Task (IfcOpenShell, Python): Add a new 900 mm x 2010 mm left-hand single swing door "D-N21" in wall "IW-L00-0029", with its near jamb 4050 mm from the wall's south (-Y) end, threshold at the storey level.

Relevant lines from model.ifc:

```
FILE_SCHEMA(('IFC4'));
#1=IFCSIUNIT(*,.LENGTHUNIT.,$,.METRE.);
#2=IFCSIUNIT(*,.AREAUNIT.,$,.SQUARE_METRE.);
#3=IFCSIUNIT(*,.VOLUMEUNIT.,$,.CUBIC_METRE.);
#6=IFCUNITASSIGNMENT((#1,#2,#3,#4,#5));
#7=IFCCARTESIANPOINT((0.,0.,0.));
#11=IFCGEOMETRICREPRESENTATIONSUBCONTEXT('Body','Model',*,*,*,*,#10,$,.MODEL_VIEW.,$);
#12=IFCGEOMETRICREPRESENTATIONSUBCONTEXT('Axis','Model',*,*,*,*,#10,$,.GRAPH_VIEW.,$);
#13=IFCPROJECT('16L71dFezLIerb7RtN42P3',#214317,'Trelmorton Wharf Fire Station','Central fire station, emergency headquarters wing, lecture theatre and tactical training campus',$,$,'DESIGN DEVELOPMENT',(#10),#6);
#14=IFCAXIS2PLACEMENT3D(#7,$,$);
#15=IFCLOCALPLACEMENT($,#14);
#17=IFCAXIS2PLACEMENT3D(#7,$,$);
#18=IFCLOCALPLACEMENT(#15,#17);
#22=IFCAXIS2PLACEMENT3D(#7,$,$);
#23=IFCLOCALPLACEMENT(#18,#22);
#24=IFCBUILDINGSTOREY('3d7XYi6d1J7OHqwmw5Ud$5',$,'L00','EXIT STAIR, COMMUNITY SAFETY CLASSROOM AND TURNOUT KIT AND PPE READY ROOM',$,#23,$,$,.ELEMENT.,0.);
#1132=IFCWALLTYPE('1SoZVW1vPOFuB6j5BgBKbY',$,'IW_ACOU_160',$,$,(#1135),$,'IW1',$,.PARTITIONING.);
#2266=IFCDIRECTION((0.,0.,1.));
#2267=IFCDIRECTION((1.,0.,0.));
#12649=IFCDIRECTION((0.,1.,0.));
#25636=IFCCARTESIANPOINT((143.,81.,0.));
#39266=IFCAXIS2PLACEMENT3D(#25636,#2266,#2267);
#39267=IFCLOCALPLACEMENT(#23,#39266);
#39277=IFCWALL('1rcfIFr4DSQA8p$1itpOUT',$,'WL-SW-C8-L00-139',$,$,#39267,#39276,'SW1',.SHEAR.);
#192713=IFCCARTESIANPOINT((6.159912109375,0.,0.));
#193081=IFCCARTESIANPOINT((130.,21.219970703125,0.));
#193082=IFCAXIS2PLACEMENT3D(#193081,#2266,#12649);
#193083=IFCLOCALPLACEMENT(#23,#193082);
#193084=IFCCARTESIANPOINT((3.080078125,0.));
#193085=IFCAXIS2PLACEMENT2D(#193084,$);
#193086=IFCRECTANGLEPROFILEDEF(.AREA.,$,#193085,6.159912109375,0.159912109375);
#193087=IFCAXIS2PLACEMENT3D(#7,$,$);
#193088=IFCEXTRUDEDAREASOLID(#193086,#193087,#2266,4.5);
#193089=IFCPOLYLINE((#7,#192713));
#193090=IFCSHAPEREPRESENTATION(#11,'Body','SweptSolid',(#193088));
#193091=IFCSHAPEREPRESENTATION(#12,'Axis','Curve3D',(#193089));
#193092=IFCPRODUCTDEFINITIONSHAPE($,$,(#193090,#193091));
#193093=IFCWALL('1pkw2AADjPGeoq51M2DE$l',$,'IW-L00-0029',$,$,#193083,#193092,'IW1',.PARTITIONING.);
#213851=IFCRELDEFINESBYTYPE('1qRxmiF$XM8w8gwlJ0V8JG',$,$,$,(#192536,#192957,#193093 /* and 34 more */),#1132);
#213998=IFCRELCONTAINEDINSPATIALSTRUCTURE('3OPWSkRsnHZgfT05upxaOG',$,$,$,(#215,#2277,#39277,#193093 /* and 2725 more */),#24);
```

```python
import numpy as np
import ifcopenshell
import ifcopenshell.api.feature
import ifcopenshell.api.geometry
import ifcopenshell.api.root
import ifcopenshell.api.spatial
import ifcopenshell.geom
import ifcopenshell.util.element
import ifcopenshell.util.placement
import ifcopenshell.util.representation
import ifcopenshell.util.shape
import ifcopenshell.util.unit

model = ifcopenshell.open("model.ifc")
unit_scale = ifcopenshell.util.unit.calculate_unit_scale(model)
settings = ifcopenshell.geom.settings()


def volume(element):
    """Net volume in cubic metres, openings subtracted."""
    shape = ifcopenshell.geom.create_shape(settings, element)
    return ifcopenshell.util.shape.get_volume(shape.geometry)


wall = model.by_guid("1pkw2AADjPGeoq51M2DE$l")
storey = ifcopenshell.util.element.get_container(wall, ifc_class="IfcBuildingStorey")
context = ifcopenshell.util.representation.get_context(model, "Model", "Body", "MODEL_VIEW")
before = volume(wall)

width, height, from_end, sill = 0.9, 2.01, 4.05, 0.0  # metres

# The wall runs along its own X axis, and the end named is its -X end.
wall_shape = ifcopenshell.geom.create_shape(settings, wall)
x, y, z = ifcopenshell.util.shape.get_vertices(wall_shape.geometry).T
start = x.min() + from_end
face, thickness = float(y.min()), float(y.max() - y.min())
wall_matrix = ifcopenshell.util.placement.get_local_placement(wall.ObjectPlacement)
level = ifcopenshell.util.placement.get_local_placement(storey.ObjectPlacement)[2, 3]


def in_wall(x, y):
    """Placement at x, y metres in the wall's axes, at sill height."""
    matrix = wall_matrix.copy()
    matrix[:, 3] = wall_matrix @ np.array([x / unit_scale, y / unit_scale, 0.0, 1.0])
    matrix[2, 3] = level + sill / unit_scale
    return matrix


# Opening: a box that overshoots both wall faces by 50 mm.
opening = ifcopenshell.api.root.create_entity(model, ifc_class="IfcOpeningElement", predefined_type="OPENING")
box = ifcopenshell.api.geometry.add_wall_representation(
    model, context=context, length=width, height=height, thickness=thickness + 0.1
)
ifcopenshell.api.geometry.assign_representation(model, product=opening, representation=box)
ifcopenshell.api.geometry.edit_object_placement(model, product=opening, matrix=in_wall(start, face - 0.05), is_si=False)
ifcopenshell.api.feature.add_feature(model, feature=opening, element=wall)

door = ifcopenshell.api.root.create_entity(model, ifc_class="IfcDoor", name="D-N21", predefined_type="DOOR")
door.OverallWidth, door.OverallHeight = width / unit_scale, height / unit_scale
door.OperationType = "SINGLE_SWING_LEFT"
body = ifcopenshell.api.geometry.add_door_representation(
    model,
    context=context,
    overall_width=door.OverallWidth,
    overall_height=door.OverallHeight,
    operation_type="SINGLE_SWING_LEFT",
    lining_properties={"LiningDepth": thickness / unit_scale, "ThresholdDepth": thickness / unit_scale},
)
ifcopenshell.api.geometry.assign_representation(model, product=door, representation=body)
ifcopenshell.api.spatial.assign_container(model, products=[door], relating_structure=storey)
ifcopenshell.api.feature.add_filling(model, opening=opening, element=door)

# The lining spans the wall, so the door starts at the wall face.
ifcopenshell.api.geometry.edit_object_placement(model, product=door, matrix=in_wall(start, face), is_si=False)

after = volume(wall)

print(f"wall volume {before:.3f} -> {after:.3f} m3")

model.write("model_updated.ifc")
```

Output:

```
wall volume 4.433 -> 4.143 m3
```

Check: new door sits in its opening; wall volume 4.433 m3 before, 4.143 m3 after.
